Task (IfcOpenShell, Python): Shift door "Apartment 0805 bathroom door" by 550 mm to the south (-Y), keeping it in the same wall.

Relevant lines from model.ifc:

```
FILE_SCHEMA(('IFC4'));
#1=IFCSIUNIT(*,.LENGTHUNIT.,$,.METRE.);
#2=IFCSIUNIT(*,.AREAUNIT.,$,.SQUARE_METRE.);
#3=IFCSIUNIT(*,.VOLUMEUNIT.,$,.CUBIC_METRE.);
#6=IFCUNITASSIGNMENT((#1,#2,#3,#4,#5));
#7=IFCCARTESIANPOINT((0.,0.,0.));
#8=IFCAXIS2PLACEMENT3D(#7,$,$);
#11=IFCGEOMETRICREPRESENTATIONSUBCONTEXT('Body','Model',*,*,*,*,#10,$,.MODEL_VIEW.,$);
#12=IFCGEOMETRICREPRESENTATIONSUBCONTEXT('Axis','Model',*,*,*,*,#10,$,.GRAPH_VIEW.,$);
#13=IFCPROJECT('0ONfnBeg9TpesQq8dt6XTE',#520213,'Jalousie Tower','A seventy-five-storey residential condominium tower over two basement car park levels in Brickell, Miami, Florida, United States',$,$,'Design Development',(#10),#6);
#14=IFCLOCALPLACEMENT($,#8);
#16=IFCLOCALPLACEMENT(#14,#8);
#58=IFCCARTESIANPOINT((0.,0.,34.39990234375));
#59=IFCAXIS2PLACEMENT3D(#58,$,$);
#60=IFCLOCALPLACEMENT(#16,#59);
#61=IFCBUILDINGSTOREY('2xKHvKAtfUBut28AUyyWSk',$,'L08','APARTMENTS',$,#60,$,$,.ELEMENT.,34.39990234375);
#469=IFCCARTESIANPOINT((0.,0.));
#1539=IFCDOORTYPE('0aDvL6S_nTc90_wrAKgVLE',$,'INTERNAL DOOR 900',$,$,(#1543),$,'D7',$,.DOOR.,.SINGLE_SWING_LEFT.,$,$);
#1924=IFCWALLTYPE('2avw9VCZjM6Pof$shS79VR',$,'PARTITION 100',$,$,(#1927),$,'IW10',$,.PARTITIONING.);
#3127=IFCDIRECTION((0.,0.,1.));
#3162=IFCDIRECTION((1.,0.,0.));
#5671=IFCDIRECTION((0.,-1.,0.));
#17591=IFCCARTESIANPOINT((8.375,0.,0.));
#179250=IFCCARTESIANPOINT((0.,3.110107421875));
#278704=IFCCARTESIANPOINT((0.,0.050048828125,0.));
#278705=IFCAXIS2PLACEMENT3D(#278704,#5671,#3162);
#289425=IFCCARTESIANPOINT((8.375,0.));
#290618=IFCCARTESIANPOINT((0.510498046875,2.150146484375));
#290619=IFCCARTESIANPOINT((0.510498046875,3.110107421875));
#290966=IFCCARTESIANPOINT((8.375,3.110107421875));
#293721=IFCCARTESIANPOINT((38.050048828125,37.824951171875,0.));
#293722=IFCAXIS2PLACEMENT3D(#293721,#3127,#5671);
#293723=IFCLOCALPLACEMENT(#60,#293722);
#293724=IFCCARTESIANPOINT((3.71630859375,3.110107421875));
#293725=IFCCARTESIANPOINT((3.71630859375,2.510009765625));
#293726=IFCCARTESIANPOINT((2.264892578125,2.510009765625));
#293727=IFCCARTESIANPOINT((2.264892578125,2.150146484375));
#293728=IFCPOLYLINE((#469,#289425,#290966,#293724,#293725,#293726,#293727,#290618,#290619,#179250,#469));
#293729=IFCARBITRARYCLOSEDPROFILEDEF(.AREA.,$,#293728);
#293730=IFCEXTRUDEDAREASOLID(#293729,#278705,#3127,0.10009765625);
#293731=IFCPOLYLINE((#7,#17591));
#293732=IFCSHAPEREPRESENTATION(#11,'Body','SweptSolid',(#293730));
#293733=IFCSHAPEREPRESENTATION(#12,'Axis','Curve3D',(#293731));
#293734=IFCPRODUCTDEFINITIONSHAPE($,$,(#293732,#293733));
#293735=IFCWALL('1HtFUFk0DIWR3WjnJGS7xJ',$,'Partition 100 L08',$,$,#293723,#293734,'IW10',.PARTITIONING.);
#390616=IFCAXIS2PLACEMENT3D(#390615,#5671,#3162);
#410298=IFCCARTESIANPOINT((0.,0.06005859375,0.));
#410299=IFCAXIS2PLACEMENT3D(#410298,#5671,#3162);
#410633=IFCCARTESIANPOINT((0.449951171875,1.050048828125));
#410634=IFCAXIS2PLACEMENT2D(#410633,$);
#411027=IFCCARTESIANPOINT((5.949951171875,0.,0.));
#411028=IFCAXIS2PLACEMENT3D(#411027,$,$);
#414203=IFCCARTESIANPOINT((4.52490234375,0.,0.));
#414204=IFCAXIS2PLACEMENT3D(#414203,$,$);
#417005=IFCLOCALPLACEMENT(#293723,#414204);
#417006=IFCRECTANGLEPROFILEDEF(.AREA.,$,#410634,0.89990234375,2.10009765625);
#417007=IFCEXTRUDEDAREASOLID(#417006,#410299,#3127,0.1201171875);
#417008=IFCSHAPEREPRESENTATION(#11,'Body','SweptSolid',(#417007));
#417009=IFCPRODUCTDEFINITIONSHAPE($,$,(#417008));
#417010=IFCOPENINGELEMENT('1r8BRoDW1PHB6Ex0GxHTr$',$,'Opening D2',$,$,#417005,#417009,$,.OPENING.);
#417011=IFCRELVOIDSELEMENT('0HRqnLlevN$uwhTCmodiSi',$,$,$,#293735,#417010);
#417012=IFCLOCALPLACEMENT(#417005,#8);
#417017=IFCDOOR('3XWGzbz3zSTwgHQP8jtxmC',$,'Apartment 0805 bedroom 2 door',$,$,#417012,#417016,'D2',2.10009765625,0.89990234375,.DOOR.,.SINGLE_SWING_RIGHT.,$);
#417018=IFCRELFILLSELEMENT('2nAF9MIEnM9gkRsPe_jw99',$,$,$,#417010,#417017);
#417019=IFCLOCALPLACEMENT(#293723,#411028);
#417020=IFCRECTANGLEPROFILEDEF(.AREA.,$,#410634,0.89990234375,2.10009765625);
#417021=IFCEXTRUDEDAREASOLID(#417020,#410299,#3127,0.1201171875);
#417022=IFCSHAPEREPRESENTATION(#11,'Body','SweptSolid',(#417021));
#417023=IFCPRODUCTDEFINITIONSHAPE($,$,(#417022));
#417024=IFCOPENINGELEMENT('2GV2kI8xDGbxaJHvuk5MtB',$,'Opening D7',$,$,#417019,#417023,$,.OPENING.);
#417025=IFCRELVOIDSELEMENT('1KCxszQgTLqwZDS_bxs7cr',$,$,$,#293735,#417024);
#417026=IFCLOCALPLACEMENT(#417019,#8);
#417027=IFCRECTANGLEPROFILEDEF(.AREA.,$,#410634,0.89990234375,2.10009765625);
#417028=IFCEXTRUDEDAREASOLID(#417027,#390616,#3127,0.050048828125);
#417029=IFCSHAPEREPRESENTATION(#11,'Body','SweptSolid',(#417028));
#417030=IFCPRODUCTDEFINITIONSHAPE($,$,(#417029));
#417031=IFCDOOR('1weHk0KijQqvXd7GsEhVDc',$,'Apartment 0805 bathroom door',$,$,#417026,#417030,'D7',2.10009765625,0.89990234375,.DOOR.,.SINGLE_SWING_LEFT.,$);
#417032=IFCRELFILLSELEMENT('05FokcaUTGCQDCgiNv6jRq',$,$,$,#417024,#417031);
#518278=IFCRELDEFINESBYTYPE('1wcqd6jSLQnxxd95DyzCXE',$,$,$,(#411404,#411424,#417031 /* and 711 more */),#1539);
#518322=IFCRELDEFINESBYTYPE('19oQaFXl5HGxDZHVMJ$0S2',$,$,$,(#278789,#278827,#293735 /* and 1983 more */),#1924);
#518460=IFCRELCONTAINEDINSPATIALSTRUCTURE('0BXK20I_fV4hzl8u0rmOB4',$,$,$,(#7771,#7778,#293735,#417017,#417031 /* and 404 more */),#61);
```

```python
import ifcopenshell
import ifcopenshell.api.geometry
import ifcopenshell.util.placement
import ifcopenshell.util.unit

model = ifcopenshell.open("model.ifc")
unit_scale = ifcopenshell.util.unit.calculate_unit_scale(model)

door = model.by_guid("1weHk0KijQqvXd7GsEhVDc")
opening = door.FillsVoids[0].RelatingOpeningElement
wall = opening.VoidsElements[0].RelatingBuildingElement

wall_matrix = ifcopenshell.util.placement.get_local_placement(wall.ObjectPlacement)
shift = wall_matrix[:3, 0] * 0.55 / unit_scale
before = ifcopenshell.util.placement.get_local_placement(door.ObjectPlacement)[:3, 3].copy()

# The door is placed relative to its opening, so it follows when the opening moves.
matrix = ifcopenshell.util.placement.get_local_placement(opening.ObjectPlacement)
matrix[:3, 3] += shift
ifcopenshell.api.geometry.edit_object_placement(
    model, product=opening, matrix=matrix, is_si=False, should_transform_children=True
)

after = ifcopenshell.util.placement.get_local_placement(door.ObjectPlacement)[:3, 3]
print("door moved by", (after - before).round(3) + 0.0)

model.write("model_updated.ifc")
```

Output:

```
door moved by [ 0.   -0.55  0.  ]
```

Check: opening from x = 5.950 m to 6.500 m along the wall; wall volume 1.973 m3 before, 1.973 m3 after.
